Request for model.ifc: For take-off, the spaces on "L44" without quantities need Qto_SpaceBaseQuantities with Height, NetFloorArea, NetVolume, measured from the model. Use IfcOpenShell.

First a look at what the model holds.

```python
import ifcopenshell
import ifcopenshell.util.element
import ifcopenshell.util.unit

model = ifcopenshell.open("model.ifc")
print(model.schema)
for unit_type in ("LENGTHUNIT", "AREAUNIT", "VOLUMEUNIT"):
    print(unit_type, ifcopenshell.util.unit.calculate_unit_scale(model, unit_type))
storey = next(s for s in model.by_type("IfcBuildingStorey") if s.Name == "L44")
spaces = [e for e in ifcopenshell.util.element.get_decomposition(storey) if e.is_a("IfcSpace")]
for e in sorted(spaces, key=lambda e: e.id()):
    print(e.id(), e.is_a(), e.Name, list(ifcopenshell.util.element.get_psets(e, qtos_only=True)), sep=" | ")
```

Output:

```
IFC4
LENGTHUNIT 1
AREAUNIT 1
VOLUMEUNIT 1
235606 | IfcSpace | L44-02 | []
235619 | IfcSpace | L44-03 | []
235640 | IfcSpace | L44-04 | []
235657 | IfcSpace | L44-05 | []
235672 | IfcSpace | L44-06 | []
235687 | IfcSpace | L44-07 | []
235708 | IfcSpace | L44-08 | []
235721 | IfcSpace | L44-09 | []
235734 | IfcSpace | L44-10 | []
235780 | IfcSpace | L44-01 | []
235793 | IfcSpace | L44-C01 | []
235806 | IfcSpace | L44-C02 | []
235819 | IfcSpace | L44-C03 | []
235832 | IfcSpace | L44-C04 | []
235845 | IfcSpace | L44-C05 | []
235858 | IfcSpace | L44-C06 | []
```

```python
import ifcopenshell
import ifcopenshell.api.pset
import ifcopenshell.geom
import ifcopenshell.util.element
import ifcopenshell.util.shape
import ifcopenshell.util.unit

model = ifcopenshell.open("model.ifc")
unit_scale = ifcopenshell.util.unit.calculate_unit_scale(model)
area_scale = ifcopenshell.util.unit.calculate_unit_scale(model, "AREAUNIT")
volume_scale = ifcopenshell.util.unit.calculate_unit_scale(model, "VOLUMEUNIT")
settings = ifcopenshell.geom.settings()

storey = next(s for s in model.by_type("IfcBuildingStorey") if s.Name == "L44")
spaces = [e for e in ifcopenshell.util.element.get_decomposition(storey) if e.is_a("IfcSpace")]

for e in sorted(spaces, key=lambda e: e.id()):
    if ifcopenshell.util.element.get_psets(e, qtos_only=True, should_inherit=False):
        continue
    # Geometry comes back in metres, in the element's own axes.
    shape = ifcopenshell.geom.create_shape(settings, e)
    values = {
        "Height": ifcopenshell.util.shape.get_z(shape.geometry) / unit_scale,
        "NetFloorArea": ifcopenshell.util.shape.get_footprint_area(shape.geometry) / area_scale,
        "NetVolume": ifcopenshell.util.shape.get_volume(shape.geometry) / volume_scale,
    }
    qto = ifcopenshell.api.pset.add_qto(model, product=e, name="Qto_SpaceBaseQuantities")
    ifcopenshell.api.pset.edit_qto(model, qto=qto, properties=values)
    print(e.id(), {k: round(v, 3) for k, v in values.items()})

model.write("model_v2.ifc")
```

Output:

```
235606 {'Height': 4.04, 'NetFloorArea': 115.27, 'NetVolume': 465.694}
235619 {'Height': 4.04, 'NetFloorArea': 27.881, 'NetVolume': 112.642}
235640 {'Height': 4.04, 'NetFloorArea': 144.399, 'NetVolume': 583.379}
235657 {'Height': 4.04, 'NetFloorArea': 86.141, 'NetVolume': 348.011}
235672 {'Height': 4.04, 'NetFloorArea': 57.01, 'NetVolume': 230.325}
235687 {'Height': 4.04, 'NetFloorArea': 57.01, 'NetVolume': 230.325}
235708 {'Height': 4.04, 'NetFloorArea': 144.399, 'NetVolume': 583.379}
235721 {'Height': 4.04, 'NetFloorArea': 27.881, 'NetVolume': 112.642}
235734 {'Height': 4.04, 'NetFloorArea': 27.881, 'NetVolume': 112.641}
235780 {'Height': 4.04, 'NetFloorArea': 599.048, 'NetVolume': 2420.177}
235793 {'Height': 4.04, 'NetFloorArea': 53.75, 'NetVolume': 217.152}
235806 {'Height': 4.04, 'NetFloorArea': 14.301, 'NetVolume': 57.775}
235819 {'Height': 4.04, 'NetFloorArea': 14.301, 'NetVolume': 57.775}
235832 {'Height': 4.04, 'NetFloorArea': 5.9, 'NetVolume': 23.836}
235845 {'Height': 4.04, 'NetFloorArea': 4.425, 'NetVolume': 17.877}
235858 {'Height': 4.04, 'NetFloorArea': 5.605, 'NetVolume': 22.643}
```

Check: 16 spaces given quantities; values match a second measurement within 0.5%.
